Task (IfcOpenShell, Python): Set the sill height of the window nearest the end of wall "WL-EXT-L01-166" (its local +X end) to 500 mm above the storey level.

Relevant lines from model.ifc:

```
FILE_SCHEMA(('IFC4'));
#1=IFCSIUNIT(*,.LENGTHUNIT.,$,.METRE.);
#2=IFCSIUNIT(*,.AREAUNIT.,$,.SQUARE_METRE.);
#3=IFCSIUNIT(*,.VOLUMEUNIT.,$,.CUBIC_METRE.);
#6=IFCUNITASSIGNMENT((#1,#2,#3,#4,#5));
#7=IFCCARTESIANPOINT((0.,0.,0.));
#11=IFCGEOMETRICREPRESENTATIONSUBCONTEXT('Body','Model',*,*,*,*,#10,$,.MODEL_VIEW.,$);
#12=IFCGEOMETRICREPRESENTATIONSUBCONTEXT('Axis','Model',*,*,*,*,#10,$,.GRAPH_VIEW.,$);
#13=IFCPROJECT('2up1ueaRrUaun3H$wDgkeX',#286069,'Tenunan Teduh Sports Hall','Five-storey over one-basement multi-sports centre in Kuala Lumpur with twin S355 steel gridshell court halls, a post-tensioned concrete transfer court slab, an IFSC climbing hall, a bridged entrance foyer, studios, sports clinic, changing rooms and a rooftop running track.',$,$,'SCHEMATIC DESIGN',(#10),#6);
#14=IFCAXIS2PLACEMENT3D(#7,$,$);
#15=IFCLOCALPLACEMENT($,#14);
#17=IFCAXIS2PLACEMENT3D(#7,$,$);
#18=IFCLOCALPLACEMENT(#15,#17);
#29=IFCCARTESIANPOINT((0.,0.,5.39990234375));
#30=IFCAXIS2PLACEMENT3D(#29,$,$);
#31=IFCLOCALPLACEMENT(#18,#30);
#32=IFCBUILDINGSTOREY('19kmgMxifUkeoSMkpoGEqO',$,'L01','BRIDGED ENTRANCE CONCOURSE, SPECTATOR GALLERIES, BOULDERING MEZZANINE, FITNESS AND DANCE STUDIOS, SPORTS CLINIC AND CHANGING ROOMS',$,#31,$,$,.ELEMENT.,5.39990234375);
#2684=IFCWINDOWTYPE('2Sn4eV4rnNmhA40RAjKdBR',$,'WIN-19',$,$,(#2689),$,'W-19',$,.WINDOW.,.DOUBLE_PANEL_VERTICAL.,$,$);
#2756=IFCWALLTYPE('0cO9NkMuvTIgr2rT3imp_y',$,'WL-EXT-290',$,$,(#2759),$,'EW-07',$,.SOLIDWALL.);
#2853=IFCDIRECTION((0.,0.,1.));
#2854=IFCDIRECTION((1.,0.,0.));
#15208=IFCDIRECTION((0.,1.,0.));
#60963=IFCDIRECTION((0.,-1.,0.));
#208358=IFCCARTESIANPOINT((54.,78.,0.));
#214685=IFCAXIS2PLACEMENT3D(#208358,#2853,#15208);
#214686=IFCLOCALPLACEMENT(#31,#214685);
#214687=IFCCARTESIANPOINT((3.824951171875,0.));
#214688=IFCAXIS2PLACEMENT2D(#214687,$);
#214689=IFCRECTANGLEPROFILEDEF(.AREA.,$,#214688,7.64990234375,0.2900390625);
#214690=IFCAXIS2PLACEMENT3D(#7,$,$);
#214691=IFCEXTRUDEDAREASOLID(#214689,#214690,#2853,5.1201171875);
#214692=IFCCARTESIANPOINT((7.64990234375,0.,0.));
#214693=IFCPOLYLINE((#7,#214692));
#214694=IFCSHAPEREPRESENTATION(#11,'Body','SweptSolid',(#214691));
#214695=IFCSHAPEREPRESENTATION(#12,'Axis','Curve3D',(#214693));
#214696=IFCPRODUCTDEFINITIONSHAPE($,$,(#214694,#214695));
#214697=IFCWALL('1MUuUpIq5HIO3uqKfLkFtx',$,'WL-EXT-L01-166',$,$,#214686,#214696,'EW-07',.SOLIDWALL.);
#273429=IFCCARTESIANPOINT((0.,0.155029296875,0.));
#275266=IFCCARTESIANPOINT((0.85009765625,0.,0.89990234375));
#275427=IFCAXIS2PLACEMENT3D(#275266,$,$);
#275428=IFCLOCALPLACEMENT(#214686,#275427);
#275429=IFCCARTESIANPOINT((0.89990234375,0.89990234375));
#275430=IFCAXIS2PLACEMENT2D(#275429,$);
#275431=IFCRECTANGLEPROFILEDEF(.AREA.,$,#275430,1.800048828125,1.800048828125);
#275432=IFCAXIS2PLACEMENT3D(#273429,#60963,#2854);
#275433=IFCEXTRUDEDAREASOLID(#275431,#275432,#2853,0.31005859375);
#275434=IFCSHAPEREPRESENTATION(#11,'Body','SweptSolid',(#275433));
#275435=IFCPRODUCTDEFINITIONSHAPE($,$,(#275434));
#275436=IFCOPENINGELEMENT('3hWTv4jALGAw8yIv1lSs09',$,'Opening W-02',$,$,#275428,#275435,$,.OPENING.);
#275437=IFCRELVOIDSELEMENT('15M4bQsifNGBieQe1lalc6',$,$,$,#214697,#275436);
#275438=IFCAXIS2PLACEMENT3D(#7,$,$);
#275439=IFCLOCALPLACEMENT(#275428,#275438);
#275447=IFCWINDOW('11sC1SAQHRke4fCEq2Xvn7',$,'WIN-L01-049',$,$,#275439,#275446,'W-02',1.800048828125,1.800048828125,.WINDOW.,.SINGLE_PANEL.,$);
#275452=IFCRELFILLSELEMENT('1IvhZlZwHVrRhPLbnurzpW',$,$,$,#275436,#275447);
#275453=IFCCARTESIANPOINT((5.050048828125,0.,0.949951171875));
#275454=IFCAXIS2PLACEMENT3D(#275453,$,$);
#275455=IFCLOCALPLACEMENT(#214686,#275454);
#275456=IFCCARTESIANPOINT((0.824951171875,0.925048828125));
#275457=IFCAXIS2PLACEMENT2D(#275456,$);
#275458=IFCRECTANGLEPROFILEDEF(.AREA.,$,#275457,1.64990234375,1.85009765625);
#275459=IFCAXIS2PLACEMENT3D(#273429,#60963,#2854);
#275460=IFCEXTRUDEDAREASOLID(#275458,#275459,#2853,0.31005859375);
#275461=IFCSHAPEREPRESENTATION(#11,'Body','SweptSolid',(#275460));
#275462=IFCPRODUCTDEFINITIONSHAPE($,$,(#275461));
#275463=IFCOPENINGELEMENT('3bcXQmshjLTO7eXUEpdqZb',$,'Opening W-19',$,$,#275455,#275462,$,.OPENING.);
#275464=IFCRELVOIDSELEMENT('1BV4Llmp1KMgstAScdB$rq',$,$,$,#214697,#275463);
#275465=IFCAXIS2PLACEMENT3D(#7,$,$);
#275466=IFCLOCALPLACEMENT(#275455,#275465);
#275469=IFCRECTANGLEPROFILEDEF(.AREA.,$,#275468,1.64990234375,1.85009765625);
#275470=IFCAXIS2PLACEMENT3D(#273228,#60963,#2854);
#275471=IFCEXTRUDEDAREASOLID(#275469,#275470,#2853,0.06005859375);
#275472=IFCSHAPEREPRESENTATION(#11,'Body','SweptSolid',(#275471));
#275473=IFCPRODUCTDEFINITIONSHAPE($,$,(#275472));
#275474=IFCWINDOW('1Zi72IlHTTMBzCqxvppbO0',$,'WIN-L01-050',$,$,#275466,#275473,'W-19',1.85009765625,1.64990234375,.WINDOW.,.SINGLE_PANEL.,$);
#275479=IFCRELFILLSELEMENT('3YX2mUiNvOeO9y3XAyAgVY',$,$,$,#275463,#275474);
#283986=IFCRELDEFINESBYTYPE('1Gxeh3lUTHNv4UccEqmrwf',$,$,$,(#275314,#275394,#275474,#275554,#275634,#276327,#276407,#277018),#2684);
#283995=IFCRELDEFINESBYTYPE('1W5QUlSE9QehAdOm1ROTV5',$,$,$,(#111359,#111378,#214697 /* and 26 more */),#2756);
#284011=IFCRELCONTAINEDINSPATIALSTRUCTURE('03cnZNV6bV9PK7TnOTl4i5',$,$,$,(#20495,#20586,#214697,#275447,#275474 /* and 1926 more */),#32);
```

```python
import numpy as np
import ifcopenshell
import ifcopenshell.api.geometry
import ifcopenshell.geom
import ifcopenshell.util.element
import ifcopenshell.util.placement
import ifcopenshell.util.shape
import ifcopenshell.util.unit

model = ifcopenshell.open("model.ifc")
unit_scale = ifcopenshell.util.unit.calculate_unit_scale(model)

window = model.by_id(275474)
opening = window.FillsVoids[0].RelatingOpeningElement
storey = ifcopenshell.util.element.get_container(window, ifc_class="IfcBuildingStorey")
level = ifcopenshell.util.placement.get_local_placement(storey.ObjectPlacement)[2, 3]

# The opening's origin need not be at the sill, so measure its lowest point.
shape = ifcopenshell.geom.create_shape(ifcopenshell.geom.settings(), opening)
bottom = ifcopenshell.util.shape.get_shape_bottom_elevation(shape, shape.geometry) / unit_scale
dz = level + 0.5 / unit_scale - bottom

shift = np.array([0.0, 0.0, dz])
# The window is placed relative to its opening, so it follows when the opening moves.
matrix = ifcopenshell.util.placement.get_local_placement(opening.ObjectPlacement)
matrix[:3, 3] += shift
ifcopenshell.api.geometry.edit_object_placement(
    model, product=opening, matrix=matrix, is_si=False, should_transform_children=True
)

print(f"moved by {dz * unit_scale:+.3f} m")

model.write("model_v2.ifc")
```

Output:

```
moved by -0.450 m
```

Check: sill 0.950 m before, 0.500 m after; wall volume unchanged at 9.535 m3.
